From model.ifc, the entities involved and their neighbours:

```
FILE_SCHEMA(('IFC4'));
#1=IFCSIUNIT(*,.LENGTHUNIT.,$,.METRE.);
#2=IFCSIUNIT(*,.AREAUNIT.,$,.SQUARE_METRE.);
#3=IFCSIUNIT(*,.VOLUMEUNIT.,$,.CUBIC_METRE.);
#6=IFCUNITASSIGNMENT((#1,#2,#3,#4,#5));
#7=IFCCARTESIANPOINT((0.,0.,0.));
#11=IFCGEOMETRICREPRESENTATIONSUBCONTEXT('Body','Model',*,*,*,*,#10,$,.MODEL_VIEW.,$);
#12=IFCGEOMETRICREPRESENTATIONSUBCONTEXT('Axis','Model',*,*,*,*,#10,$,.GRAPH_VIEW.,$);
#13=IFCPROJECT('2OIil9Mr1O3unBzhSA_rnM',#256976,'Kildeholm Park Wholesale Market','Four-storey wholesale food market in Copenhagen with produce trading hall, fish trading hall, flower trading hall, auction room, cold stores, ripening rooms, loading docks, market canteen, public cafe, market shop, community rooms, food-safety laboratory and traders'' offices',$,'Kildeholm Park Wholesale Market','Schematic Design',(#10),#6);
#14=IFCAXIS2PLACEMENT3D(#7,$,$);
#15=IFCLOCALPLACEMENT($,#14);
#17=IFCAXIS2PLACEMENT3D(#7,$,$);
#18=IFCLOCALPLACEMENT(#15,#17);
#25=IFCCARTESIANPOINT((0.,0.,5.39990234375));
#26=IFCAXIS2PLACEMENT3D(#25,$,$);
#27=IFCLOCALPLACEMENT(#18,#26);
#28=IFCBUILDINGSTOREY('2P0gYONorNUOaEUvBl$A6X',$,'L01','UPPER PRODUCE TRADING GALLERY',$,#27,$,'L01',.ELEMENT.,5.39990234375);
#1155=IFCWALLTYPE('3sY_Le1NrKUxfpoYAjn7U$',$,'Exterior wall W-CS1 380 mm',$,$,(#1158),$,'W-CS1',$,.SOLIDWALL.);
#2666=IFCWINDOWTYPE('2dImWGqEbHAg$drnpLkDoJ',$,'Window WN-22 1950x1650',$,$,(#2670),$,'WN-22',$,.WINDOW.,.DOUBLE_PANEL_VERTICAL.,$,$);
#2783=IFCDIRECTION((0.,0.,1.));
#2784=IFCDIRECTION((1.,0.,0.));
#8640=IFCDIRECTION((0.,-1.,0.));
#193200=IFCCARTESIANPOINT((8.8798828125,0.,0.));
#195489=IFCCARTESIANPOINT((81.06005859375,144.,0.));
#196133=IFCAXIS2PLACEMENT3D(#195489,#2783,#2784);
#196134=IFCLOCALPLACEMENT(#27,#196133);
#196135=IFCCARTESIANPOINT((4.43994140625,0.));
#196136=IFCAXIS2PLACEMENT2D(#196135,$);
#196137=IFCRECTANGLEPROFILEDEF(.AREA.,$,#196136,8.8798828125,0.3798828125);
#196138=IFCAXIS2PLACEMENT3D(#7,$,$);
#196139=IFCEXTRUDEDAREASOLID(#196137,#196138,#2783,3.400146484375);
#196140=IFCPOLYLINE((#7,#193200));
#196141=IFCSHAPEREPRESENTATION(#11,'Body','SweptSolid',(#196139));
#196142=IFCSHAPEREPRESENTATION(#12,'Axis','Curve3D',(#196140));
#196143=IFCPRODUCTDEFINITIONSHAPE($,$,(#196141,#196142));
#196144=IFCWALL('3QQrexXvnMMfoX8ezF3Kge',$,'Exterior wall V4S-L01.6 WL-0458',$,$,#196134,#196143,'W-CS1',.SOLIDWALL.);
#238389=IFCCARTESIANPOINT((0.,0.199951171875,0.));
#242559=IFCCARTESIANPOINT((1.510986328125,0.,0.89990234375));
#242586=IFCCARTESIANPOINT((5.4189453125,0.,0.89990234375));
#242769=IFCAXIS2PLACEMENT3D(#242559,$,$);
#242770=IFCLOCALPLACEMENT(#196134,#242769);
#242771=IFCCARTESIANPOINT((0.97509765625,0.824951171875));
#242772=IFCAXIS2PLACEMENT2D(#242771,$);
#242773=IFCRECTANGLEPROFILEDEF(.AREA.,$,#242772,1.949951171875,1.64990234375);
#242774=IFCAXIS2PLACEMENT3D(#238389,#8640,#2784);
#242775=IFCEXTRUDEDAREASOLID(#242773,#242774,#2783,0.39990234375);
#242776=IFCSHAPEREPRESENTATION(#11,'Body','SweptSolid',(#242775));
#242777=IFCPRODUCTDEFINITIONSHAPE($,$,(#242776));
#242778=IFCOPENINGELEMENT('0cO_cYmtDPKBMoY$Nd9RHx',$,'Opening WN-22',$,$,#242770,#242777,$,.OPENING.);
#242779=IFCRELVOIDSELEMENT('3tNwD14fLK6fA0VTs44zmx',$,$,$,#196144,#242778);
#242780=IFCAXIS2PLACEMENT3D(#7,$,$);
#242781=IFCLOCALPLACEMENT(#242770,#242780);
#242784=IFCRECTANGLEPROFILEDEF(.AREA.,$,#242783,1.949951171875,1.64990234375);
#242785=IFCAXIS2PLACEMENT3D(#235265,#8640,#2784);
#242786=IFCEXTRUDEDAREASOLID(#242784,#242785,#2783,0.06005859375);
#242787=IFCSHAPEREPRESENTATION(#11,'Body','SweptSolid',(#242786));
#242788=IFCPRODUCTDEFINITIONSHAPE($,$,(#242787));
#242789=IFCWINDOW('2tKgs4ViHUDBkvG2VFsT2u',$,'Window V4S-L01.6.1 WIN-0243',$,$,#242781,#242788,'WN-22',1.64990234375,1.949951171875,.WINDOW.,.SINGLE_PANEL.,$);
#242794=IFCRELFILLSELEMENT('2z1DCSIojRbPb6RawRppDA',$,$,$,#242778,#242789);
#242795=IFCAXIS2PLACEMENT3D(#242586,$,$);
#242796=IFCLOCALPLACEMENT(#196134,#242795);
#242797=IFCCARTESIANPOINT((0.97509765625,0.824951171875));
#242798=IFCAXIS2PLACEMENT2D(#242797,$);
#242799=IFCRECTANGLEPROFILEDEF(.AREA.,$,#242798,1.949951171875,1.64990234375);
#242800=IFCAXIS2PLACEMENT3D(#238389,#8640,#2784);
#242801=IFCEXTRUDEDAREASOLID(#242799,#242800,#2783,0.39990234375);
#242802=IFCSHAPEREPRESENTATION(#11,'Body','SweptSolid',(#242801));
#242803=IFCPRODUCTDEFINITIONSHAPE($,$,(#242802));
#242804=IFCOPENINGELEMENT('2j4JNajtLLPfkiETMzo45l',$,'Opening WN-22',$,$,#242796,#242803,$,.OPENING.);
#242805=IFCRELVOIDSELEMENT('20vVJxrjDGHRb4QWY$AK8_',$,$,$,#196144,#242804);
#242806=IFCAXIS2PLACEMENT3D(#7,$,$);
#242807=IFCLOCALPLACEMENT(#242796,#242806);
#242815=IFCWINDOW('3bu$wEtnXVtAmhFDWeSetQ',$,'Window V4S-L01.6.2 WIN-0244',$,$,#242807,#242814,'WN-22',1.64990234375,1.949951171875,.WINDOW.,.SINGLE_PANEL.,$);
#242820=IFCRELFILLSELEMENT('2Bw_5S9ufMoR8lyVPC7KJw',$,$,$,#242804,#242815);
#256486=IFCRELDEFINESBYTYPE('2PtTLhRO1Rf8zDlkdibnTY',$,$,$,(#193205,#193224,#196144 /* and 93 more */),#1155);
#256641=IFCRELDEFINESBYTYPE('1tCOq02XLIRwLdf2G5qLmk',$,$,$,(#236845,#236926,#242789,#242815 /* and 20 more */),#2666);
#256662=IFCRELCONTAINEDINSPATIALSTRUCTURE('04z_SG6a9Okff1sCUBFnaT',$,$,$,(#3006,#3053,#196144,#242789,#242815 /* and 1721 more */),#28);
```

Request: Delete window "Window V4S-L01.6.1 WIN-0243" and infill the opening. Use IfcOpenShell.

```python
import ifcopenshell
import ifcopenshell.api.feature
import ifcopenshell.api.root
import ifcopenshell.geom
import ifcopenshell.util.shape

model = ifcopenshell.open("model.ifc")
settings = ifcopenshell.geom.settings()


def volume(element):
    """Net volume in cubic metres, openings subtracted."""
    shape = ifcopenshell.geom.create_shape(settings, element)
    return ifcopenshell.util.shape.get_volume(shape.geometry)


window = model.by_guid("2tKgs4ViHUDBkvG2VFsT2u")
opening = window.FillsVoids[0].RelatingOpeningElement
wall = opening.VoidsElements[0].RelatingBuildingElement
before = volume(wall)

ifcopenshell.api.root.remove_product(model, product=window)
ifcopenshell.api.feature.remove_feature(model, feature=opening)

after = volume(wall)

print(f"wall volume {before:.3f} -> {after:.3f} m3")

model.write("model_edited.ifc")
```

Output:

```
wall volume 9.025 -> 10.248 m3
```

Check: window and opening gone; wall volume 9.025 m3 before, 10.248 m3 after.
